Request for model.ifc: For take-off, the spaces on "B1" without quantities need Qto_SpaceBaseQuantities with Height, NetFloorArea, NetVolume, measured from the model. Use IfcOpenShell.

First a look at what the model holds.

```python
import ifcopenshell
import ifcopenshell.util.element
import ifcopenshell.util.unit

model = ifcopenshell.open("model.ifc")
print(model.schema)
for unit_type in ("LENGTHUNIT", "AREAUNIT", "VOLUMEUNIT"):
    print(unit_type, ifcopenshell.util.unit.calculate_unit_scale(model, unit_type))
storey = next(s for s in model.by_type("IfcBuildingStorey") if s.Name == "B1")
spaces = [e for e in ifcopenshell.util.element.get_decomposition(storey) if e.is_a("IfcSpace")]
for e in sorted(spaces, key=lambda e: e.id()):
    print(e.id(), e.is_a(), e.Name, list(ifcopenshell.util.element.get_psets(e, qtos_only=True)), sep=" | ")
```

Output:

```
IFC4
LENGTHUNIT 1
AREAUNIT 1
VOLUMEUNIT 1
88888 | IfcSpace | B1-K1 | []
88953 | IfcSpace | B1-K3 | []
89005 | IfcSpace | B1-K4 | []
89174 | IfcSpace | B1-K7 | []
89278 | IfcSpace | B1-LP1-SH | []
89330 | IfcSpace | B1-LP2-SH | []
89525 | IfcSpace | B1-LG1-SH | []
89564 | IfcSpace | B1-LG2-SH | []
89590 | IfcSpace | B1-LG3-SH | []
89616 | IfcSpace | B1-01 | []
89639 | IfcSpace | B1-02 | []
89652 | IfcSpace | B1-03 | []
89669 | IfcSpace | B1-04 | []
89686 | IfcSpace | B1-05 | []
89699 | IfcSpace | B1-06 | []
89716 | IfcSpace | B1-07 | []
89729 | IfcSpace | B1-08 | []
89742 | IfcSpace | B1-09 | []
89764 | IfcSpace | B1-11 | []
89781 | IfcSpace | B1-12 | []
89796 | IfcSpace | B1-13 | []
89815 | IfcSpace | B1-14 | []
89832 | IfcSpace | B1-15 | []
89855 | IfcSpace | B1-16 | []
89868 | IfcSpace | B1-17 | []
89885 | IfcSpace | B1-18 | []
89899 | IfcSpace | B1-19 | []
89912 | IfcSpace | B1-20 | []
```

```python
import ifcopenshell
import ifcopenshell.api.pset
import ifcopenshell.geom
import ifcopenshell.util.element
import ifcopenshell.util.shape
import ifcopenshell.util.unit

model = ifcopenshell.open("model.ifc")
unit_scale = ifcopenshell.util.unit.calculate_unit_scale(model)
area_scale = ifcopenshell.util.unit.calculate_unit_scale(model, "AREAUNIT")
volume_scale = ifcopenshell.util.unit.calculate_unit_scale(model, "VOLUMEUNIT")
settings = ifcopenshell.geom.settings()

storey = next(s for s in model.by_type("IfcBuildingStorey") if s.Name == "B1")
spaces = [e for e in ifcopenshell.util.element.get_decomposition(storey) if e.is_a("IfcSpace")]

for e in sorted(spaces, key=lambda e: e.id()):
    if ifcopenshell.util.element.get_psets(e, qtos_only=True, should_inherit=False):
        continue
    # Geometry comes back in metres, in the element's own axes.
    shape = ifcopenshell.geom.create_shape(settings, e)
    values = {
        "Height": ifcopenshell.util.shape.get_z(shape.geometry) / unit_scale,
        "NetFloorArea": ifcopenshell.util.shape.get_footprint_area(shape.geometry) / area_scale,
        "NetVolume": ifcopenshell.util.shape.get_volume(shape.geometry) / volume_scale,
    }
    qto = ifcopenshell.api.pset.add_qto(model, product=e, name="Qto_SpaceBaseQuantities")
    ifcopenshell.api.pset.edit_qto(model, qto=qto, properties=values)
    print(e.id(), {k: round(v, 3) for k, v in values.items()})

model.write("model_updated.ifc")
```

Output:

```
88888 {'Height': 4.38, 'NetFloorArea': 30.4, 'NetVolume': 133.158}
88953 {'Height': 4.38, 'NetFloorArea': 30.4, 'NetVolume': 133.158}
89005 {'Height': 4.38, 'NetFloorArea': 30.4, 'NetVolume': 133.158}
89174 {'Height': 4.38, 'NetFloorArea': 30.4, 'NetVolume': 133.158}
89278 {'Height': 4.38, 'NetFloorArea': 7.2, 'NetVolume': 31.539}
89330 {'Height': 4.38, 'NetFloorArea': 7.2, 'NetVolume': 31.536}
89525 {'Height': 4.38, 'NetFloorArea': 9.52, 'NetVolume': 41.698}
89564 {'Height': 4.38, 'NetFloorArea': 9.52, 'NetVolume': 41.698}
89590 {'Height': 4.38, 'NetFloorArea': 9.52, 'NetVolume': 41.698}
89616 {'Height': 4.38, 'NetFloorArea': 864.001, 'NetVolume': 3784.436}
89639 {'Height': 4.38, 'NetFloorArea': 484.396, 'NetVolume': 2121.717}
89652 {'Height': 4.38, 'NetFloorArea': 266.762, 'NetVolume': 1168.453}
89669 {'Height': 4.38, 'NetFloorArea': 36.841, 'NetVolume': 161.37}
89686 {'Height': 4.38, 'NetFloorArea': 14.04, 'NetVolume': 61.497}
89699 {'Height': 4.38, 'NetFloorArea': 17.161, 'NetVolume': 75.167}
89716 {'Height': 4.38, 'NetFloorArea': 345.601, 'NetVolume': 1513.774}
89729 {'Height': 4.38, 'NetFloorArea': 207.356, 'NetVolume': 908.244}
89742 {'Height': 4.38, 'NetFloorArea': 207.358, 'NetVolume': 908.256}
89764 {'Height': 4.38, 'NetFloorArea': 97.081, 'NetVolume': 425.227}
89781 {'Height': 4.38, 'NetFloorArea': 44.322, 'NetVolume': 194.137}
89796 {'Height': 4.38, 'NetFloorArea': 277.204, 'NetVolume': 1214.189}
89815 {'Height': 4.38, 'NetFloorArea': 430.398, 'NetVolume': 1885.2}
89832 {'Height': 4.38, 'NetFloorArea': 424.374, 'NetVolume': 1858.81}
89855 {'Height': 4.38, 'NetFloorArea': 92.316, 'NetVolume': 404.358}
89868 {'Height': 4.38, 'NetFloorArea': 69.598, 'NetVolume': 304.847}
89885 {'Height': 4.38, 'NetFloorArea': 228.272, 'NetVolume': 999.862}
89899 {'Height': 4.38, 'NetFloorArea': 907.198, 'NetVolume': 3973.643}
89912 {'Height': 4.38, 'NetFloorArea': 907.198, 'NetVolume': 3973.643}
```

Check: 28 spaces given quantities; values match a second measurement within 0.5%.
